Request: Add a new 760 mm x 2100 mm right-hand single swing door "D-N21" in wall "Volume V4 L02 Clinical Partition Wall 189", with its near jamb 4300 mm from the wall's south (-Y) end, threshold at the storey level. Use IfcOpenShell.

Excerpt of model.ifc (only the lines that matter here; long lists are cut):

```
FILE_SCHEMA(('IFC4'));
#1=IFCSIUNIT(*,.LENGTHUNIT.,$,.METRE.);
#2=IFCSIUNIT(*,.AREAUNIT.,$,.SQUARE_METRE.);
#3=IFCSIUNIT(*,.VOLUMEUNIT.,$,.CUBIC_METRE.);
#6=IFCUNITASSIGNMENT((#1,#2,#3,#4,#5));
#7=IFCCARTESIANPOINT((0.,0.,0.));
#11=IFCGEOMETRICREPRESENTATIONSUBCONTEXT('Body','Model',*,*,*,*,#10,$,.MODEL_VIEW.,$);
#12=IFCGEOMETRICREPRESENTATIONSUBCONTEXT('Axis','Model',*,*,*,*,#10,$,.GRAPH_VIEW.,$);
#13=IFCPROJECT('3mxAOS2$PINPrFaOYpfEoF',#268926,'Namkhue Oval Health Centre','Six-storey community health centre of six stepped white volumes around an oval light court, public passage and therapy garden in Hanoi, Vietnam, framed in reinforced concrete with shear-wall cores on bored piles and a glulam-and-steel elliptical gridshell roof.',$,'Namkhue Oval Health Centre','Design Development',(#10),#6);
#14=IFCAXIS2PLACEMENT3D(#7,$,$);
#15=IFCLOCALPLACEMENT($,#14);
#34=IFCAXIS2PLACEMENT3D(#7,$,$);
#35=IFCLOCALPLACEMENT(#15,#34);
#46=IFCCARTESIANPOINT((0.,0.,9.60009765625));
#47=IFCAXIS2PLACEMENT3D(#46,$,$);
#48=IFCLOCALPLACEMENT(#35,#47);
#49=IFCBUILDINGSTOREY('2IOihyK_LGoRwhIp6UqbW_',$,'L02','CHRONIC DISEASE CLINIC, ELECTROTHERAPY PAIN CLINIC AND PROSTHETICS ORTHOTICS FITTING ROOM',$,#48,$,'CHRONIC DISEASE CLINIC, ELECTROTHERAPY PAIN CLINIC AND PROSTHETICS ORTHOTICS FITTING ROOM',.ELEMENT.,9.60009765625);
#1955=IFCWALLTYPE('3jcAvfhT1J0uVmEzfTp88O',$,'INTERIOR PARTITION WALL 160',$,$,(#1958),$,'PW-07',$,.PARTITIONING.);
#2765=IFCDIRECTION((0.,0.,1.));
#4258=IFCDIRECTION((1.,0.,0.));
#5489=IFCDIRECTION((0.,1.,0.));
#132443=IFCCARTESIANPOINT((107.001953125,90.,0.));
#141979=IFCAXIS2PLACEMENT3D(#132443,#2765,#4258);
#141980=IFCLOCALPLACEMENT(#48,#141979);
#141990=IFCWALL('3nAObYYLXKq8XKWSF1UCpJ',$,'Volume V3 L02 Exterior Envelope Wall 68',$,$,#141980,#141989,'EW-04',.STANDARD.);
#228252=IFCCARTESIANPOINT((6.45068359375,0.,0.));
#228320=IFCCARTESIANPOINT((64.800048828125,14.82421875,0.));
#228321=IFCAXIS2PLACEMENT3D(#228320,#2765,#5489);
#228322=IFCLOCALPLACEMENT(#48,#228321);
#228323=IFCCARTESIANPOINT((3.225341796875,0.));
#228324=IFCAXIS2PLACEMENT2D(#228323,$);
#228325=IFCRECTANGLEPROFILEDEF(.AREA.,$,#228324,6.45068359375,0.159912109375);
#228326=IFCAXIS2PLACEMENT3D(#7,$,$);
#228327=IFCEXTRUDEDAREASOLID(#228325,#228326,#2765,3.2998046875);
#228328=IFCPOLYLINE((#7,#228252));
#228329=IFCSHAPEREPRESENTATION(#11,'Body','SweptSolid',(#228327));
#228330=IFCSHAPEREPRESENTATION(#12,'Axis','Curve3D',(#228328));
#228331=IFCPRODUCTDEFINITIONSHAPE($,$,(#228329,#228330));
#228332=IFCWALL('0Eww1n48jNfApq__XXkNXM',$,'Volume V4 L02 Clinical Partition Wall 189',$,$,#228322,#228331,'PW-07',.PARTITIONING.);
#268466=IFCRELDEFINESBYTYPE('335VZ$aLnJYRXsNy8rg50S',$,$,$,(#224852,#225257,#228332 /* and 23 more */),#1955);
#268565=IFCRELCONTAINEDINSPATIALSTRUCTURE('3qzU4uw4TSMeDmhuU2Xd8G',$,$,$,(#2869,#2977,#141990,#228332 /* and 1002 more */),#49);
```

```python
import numpy as np
import ifcopenshell
import ifcopenshell.api.feature
import ifcopenshell.api.geometry
import ifcopenshell.api.root
import ifcopenshell.api.spatial
import ifcopenshell.geom
import ifcopenshell.util.element
import ifcopenshell.util.placement
import ifcopenshell.util.representation
import ifcopenshell.util.shape
import ifcopenshell.util.unit

model = ifcopenshell.open("model.ifc")
unit_scale = ifcopenshell.util.unit.calculate_unit_scale(model)
settings = ifcopenshell.geom.settings()


def volume(element):
    """Net volume in cubic metres, openings subtracted."""
    shape = ifcopenshell.geom.create_shape(settings, element)
    return ifcopenshell.util.shape.get_volume(shape.geometry)


wall = model.by_id(228332)
storey = ifcopenshell.util.element.get_container(wall, ifc_class="IfcBuildingStorey")
context = ifcopenshell.util.representation.get_context(model, "Model", "Body", "MODEL_VIEW")
before = volume(wall)

width, height, from_end, sill = 0.76, 2.1, 4.3, 0.0  # metres

# The wall runs along its own X axis, and the end named is its -X end.
wall_shape = ifcopenshell.geom.create_shape(settings, wall)
x, y, z = ifcopenshell.util.shape.get_vertices(wall_shape.geometry).T
start = x.min() + from_end
face, thickness = float(y.min()), float(y.max() - y.min())
wall_matrix = ifcopenshell.util.placement.get_local_placement(wall.ObjectPlacement)
level = ifcopenshell.util.placement.get_local_placement(storey.ObjectPlacement)[2, 3]


def in_wall(x, y):
    """Placement at x, y metres in the wall's axes, at sill height."""
    matrix = wall_matrix.copy()
    matrix[:, 3] = wall_matrix @ np.array([x / unit_scale, y / unit_scale, 0.0, 1.0])
    matrix[2, 3] = level + sill / unit_scale
    return matrix


# Opening: a box that overshoots both wall faces by 50 mm.
opening = ifcopenshell.api.root.create_entity(model, ifc_class="IfcOpeningElement", predefined_type="OPENING")
box = ifcopenshell.api.geometry.add_wall_representation(
    model, context=context, length=width, height=height, thickness=thickness + 0.1
)
ifcopenshell.api.geometry.assign_representation(model, product=opening, representation=box)
ifcopenshell.api.geometry.edit_object_placement(model, product=opening, matrix=in_wall(start, face - 0.05), is_si=False)
ifcopenshell.api.feature.add_feature(model, feature=opening, element=wall)

door = ifcopenshell.api.root.create_entity(model, ifc_class="IfcDoor", name="D-N21", predefined_type="DOOR")
door.OverallWidth, door.OverallHeight = width / unit_scale, height / unit_scale
door.OperationType = "SINGLE_SWING_RIGHT"
body = ifcopenshell.api.geometry.add_door_representation(
    model,
    context=context,
    overall_width=door.OverallWidth,
    overall_height=door.OverallHeight,
    operation_type="SINGLE_SWING_RIGHT",
    lining_properties={"LiningDepth": thickness / unit_scale, "ThresholdDepth": thickness / unit_scale},
)
ifcopenshell.api.geometry.assign_representation(model, product=door, representation=body)
ifcopenshell.api.spatial.assign_container(model, products=[door], relating_structure=storey)
ifcopenshell.api.feature.add_filling(model, opening=opening, element=door)

# The lining spans the wall, so the door starts at the wall face.
ifcopenshell.api.geometry.edit_object_placement(model, product=door, matrix=in_wall(start, face), is_si=False)

after = volume(wall)

print(f"wall volume {before:.3f} -> {after:.3f} m3")

model.write("model_v2.ifc")
```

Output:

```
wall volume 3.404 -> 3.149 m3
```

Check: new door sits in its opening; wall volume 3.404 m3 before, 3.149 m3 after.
